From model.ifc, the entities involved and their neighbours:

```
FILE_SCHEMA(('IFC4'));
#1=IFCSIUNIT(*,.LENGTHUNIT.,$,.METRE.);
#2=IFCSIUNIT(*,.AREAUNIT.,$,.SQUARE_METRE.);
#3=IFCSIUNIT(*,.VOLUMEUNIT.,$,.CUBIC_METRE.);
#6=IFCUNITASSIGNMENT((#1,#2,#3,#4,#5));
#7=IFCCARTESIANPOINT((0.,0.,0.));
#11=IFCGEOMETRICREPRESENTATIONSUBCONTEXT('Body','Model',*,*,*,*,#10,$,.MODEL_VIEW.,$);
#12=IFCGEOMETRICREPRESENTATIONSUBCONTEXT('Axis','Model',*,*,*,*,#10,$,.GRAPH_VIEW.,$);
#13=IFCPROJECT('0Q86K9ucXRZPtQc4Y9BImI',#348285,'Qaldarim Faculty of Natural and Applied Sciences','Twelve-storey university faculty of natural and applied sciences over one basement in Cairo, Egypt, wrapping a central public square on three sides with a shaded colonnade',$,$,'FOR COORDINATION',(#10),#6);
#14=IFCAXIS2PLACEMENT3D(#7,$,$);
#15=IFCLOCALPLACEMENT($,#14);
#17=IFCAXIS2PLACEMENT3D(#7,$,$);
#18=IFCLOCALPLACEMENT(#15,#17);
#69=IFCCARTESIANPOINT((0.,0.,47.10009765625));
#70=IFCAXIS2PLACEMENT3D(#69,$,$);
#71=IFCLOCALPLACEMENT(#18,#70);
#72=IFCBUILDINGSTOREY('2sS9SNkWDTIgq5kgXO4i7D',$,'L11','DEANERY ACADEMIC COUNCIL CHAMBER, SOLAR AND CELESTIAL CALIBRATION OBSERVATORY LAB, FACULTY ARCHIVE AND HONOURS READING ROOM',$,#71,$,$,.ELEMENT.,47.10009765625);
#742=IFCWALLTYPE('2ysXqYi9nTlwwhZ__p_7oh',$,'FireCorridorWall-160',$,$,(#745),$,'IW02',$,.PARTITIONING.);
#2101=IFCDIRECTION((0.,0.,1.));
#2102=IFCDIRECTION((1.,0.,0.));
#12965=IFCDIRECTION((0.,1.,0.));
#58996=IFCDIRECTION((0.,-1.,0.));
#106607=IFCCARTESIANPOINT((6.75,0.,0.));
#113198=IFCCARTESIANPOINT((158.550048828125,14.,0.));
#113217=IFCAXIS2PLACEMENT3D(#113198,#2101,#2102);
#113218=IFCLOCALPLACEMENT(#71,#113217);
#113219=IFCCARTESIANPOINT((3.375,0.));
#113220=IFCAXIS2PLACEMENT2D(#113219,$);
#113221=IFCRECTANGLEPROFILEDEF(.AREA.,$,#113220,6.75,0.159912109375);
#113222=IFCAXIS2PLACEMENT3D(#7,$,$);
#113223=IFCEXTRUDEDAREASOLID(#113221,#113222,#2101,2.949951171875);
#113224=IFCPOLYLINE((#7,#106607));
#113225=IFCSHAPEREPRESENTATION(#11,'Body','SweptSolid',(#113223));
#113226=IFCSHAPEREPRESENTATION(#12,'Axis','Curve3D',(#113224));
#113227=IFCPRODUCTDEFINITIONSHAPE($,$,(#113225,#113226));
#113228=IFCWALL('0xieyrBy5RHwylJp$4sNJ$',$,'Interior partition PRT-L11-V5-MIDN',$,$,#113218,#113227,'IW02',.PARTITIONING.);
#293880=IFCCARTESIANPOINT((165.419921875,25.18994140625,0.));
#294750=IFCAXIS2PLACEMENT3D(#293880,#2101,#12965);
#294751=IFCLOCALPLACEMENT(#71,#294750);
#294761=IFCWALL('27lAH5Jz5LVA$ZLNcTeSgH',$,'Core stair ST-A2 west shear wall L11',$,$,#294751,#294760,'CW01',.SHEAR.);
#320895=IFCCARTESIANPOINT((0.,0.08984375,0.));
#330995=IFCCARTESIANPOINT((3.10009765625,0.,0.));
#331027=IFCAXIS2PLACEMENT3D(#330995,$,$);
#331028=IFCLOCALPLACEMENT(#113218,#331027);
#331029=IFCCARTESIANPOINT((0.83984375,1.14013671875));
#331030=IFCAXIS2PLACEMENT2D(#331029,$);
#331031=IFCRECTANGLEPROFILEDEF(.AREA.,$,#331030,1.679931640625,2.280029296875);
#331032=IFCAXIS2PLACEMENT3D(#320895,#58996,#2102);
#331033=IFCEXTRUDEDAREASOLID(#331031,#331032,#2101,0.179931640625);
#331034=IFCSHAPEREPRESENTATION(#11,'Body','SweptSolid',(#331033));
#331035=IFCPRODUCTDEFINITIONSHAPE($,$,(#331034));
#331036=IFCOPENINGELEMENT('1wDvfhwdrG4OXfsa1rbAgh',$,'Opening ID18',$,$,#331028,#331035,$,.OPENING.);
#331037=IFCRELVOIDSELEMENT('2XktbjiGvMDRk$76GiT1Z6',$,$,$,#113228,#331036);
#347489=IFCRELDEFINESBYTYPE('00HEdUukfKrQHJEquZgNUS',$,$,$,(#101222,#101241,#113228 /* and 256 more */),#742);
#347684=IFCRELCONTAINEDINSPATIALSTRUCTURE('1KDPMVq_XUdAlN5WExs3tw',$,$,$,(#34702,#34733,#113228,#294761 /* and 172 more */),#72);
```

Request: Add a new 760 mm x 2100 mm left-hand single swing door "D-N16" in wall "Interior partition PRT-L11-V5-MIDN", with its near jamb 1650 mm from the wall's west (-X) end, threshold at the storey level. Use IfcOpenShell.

```python
import numpy as np
import ifcopenshell
import ifcopenshell.api.feature
import ifcopenshell.api.geometry
import ifcopenshell.api.root
import ifcopenshell.api.spatial
import ifcopenshell.geom
import ifcopenshell.util.element
import ifcopenshell.util.placement
import ifcopenshell.util.representation
import ifcopenshell.util.shape
import ifcopenshell.util.unit

model = ifcopenshell.open("model.ifc")
unit_scale = ifcopenshell.util.unit.calculate_unit_scale(model)
settings = ifcopenshell.geom.settings()


def volume(element):
    """Net volume in cubic metres, openings subtracted."""
    shape = ifcopenshell.geom.create_shape(settings, element)
    return ifcopenshell.util.shape.get_volume(shape.geometry)


wall = model.by_guid("0xieyrBy5RHwylJp$4sNJ$")
storey = ifcopenshell.util.element.get_container(wall, ifc_class="IfcBuildingStorey")
context = ifcopenshell.util.representation.get_context(model, "Model", "Body", "MODEL_VIEW")
before = volume(wall)

width, height, from_end, sill = 0.76, 2.1, 1.65, 0.0  # metres

# The wall runs along its own X axis, and the end named is its -X end.
wall_shape = ifcopenshell.geom.create_shape(settings, wall)
x, y, z = ifcopenshell.util.shape.get_vertices(wall_shape.geometry).T
start = x.min() + from_end
face, thickness = float(y.min()), float(y.max() - y.min())
wall_matrix = ifcopenshell.util.placement.get_local_placement(wall.ObjectPlacement)
level = ifcopenshell.util.placement.get_local_placement(storey.ObjectPlacement)[2, 3]


def in_wall(x, y):
    """Placement at x, y metres in the wall's axes, at sill height."""
    matrix = wall_matrix.copy()
    matrix[:, 3] = wall_matrix @ np.array([x / unit_scale, y / unit_scale, 0.0, 1.0])
    matrix[2, 3] = level + sill / unit_scale
    return matrix


# Opening: a box that overshoots both wall faces by 50 mm.
opening = ifcopenshell.api.root.create_entity(model, ifc_class="IfcOpeningElement", predefined_type="OPENING")
box = ifcopenshell.api.geometry.add_wall_representation(
    model, context=context, length=width, height=height, thickness=thickness + 0.1
)
ifcopenshell.api.geometry.assign_representation(model, product=opening, representation=box)
ifcopenshell.api.geometry.edit_object_placement(model, product=opening, matrix=in_wall(start, face - 0.05), is_si=False)
ifcopenshell.api.feature.add_feature(model, feature=opening, element=wall)

door = ifcopenshell.api.root.create_entity(model, ifc_class="IfcDoor", name="D-N16", predefined_type="DOOR")
door.OverallWidth, door.OverallHeight = width / unit_scale, height / unit_scale
door.OperationType = "SINGLE_SWING_LEFT"
body = ifcopenshell.api.geometry.add_door_representation(
    model,
    context=context,
    overall_width=door.OverallWidth,
    overall_height=door.OverallHeight,
    operation_type="SINGLE_SWING_LEFT",
    lining_properties={"LiningDepth": thickness / unit_scale, "ThresholdDepth": thickness / unit_scale},
)
ifcopenshell.api.geometry.assign_representation(model, product=door, representation=body)
ifcopenshell.api.spatial.assign_container(model, products=[door], relating_structure=storey)
ifcopenshell.api.feature.add_filling(model, opening=opening, element=door)

# The lining spans the wall, so the door starts at the wall face.
ifcopenshell.api.geometry.edit_object_placement(model, product=door, matrix=in_wall(start, face), is_si=False)

after = volume(wall)

print(f"wall volume {before:.3f} -> {after:.3f} m3")

model.write("model_updated.ifc")
```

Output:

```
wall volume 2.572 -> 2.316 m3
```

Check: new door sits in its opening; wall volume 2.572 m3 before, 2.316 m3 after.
